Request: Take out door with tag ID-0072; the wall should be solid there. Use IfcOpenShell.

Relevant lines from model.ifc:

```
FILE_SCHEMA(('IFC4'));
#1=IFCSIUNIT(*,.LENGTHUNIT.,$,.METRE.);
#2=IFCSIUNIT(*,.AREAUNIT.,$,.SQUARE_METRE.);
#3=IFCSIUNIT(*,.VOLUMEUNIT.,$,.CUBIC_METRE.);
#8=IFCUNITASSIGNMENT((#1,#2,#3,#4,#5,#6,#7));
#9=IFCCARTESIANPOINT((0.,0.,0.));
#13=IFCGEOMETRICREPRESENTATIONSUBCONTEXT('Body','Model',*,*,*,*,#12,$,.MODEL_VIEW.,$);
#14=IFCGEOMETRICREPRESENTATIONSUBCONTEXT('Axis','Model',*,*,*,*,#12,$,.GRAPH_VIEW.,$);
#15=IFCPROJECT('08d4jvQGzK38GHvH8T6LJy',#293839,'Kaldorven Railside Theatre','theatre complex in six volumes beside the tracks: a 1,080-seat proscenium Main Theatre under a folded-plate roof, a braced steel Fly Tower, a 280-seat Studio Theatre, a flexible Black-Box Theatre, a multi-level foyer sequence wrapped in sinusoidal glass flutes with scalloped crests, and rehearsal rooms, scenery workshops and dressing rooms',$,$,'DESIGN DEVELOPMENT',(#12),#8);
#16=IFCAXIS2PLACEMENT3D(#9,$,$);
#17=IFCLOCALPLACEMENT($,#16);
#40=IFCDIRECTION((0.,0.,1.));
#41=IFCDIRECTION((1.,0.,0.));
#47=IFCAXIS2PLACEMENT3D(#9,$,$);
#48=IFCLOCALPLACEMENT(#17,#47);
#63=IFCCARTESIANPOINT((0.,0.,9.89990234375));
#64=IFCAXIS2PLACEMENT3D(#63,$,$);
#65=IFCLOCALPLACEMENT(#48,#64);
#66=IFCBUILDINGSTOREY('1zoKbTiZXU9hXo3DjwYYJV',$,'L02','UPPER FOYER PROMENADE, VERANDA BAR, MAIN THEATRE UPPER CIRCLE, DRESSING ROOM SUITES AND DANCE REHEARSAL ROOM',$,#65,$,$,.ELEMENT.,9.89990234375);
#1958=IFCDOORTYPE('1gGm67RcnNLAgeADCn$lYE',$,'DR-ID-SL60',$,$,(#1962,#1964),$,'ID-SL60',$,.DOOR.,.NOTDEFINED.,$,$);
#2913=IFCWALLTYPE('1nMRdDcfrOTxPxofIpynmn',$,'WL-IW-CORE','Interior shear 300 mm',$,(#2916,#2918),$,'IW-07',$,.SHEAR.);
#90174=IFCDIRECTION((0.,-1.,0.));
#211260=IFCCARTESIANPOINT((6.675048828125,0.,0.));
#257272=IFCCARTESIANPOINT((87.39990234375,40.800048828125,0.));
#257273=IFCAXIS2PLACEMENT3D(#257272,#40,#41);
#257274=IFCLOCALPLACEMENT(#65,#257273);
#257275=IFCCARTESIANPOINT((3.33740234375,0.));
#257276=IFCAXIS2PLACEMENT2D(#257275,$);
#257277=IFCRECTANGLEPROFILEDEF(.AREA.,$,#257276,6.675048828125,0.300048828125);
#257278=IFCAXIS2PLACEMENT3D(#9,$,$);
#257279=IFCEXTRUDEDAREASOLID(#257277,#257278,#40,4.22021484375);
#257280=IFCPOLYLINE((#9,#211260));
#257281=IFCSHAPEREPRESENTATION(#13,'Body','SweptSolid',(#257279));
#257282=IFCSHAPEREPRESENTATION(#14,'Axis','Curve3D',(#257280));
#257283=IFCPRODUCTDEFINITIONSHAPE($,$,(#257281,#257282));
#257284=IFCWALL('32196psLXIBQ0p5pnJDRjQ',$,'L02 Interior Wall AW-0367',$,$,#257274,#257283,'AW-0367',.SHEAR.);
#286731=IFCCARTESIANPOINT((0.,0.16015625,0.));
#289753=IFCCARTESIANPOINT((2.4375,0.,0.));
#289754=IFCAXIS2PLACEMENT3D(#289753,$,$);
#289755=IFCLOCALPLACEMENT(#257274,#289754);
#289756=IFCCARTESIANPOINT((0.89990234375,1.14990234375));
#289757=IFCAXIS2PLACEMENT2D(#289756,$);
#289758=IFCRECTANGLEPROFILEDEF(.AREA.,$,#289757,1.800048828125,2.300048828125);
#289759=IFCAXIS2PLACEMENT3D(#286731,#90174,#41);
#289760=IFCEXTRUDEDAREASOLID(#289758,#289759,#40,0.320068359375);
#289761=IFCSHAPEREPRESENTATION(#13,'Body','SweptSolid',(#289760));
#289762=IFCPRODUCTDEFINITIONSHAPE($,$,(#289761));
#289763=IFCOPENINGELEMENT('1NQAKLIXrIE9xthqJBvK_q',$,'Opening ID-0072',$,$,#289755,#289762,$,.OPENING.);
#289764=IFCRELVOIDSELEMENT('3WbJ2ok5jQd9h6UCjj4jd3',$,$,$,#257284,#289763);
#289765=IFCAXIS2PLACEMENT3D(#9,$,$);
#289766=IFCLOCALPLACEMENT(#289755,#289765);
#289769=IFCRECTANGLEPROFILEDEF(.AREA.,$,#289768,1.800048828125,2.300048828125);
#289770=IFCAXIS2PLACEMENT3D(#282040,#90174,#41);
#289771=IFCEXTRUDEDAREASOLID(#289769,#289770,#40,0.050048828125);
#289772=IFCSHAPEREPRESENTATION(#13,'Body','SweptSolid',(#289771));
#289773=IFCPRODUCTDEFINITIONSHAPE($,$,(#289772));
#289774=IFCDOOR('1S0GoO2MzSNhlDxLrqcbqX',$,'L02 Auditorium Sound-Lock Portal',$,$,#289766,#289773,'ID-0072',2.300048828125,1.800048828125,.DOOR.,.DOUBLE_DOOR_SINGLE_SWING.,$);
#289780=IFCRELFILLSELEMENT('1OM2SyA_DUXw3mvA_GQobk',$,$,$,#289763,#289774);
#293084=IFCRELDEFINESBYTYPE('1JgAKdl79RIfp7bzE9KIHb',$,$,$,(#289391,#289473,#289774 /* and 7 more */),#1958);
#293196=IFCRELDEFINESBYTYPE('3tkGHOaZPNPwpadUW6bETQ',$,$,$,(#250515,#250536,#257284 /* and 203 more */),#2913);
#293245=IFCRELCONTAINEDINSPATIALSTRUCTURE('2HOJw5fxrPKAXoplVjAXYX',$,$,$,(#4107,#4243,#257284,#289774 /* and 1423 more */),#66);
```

```python
import ifcopenshell
import ifcopenshell.api.feature
import ifcopenshell.api.root
import ifcopenshell.geom
import ifcopenshell.util.shape

model = ifcopenshell.open("model.ifc")
settings = ifcopenshell.geom.settings()


def volume(element):
    """Net volume in cubic metres, openings subtracted."""
    shape = ifcopenshell.geom.create_shape(settings, element)
    return ifcopenshell.util.shape.get_volume(shape.geometry)


door = model.by_guid("1S0GoO2MzSNhlDxLrqcbqX")
opening = door.FillsVoids[0].RelatingOpeningElement
wall = opening.VoidsElements[0].RelatingBuildingElement
before = volume(wall)

ifcopenshell.api.root.remove_product(model, product=door)
ifcopenshell.api.feature.remove_feature(model, feature=opening)

after = volume(wall)

print(f"wall volume {before:.3f} -> {after:.3f} m3")

model.write("model_edited.ifc")
```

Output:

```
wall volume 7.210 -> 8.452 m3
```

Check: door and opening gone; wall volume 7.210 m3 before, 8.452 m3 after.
